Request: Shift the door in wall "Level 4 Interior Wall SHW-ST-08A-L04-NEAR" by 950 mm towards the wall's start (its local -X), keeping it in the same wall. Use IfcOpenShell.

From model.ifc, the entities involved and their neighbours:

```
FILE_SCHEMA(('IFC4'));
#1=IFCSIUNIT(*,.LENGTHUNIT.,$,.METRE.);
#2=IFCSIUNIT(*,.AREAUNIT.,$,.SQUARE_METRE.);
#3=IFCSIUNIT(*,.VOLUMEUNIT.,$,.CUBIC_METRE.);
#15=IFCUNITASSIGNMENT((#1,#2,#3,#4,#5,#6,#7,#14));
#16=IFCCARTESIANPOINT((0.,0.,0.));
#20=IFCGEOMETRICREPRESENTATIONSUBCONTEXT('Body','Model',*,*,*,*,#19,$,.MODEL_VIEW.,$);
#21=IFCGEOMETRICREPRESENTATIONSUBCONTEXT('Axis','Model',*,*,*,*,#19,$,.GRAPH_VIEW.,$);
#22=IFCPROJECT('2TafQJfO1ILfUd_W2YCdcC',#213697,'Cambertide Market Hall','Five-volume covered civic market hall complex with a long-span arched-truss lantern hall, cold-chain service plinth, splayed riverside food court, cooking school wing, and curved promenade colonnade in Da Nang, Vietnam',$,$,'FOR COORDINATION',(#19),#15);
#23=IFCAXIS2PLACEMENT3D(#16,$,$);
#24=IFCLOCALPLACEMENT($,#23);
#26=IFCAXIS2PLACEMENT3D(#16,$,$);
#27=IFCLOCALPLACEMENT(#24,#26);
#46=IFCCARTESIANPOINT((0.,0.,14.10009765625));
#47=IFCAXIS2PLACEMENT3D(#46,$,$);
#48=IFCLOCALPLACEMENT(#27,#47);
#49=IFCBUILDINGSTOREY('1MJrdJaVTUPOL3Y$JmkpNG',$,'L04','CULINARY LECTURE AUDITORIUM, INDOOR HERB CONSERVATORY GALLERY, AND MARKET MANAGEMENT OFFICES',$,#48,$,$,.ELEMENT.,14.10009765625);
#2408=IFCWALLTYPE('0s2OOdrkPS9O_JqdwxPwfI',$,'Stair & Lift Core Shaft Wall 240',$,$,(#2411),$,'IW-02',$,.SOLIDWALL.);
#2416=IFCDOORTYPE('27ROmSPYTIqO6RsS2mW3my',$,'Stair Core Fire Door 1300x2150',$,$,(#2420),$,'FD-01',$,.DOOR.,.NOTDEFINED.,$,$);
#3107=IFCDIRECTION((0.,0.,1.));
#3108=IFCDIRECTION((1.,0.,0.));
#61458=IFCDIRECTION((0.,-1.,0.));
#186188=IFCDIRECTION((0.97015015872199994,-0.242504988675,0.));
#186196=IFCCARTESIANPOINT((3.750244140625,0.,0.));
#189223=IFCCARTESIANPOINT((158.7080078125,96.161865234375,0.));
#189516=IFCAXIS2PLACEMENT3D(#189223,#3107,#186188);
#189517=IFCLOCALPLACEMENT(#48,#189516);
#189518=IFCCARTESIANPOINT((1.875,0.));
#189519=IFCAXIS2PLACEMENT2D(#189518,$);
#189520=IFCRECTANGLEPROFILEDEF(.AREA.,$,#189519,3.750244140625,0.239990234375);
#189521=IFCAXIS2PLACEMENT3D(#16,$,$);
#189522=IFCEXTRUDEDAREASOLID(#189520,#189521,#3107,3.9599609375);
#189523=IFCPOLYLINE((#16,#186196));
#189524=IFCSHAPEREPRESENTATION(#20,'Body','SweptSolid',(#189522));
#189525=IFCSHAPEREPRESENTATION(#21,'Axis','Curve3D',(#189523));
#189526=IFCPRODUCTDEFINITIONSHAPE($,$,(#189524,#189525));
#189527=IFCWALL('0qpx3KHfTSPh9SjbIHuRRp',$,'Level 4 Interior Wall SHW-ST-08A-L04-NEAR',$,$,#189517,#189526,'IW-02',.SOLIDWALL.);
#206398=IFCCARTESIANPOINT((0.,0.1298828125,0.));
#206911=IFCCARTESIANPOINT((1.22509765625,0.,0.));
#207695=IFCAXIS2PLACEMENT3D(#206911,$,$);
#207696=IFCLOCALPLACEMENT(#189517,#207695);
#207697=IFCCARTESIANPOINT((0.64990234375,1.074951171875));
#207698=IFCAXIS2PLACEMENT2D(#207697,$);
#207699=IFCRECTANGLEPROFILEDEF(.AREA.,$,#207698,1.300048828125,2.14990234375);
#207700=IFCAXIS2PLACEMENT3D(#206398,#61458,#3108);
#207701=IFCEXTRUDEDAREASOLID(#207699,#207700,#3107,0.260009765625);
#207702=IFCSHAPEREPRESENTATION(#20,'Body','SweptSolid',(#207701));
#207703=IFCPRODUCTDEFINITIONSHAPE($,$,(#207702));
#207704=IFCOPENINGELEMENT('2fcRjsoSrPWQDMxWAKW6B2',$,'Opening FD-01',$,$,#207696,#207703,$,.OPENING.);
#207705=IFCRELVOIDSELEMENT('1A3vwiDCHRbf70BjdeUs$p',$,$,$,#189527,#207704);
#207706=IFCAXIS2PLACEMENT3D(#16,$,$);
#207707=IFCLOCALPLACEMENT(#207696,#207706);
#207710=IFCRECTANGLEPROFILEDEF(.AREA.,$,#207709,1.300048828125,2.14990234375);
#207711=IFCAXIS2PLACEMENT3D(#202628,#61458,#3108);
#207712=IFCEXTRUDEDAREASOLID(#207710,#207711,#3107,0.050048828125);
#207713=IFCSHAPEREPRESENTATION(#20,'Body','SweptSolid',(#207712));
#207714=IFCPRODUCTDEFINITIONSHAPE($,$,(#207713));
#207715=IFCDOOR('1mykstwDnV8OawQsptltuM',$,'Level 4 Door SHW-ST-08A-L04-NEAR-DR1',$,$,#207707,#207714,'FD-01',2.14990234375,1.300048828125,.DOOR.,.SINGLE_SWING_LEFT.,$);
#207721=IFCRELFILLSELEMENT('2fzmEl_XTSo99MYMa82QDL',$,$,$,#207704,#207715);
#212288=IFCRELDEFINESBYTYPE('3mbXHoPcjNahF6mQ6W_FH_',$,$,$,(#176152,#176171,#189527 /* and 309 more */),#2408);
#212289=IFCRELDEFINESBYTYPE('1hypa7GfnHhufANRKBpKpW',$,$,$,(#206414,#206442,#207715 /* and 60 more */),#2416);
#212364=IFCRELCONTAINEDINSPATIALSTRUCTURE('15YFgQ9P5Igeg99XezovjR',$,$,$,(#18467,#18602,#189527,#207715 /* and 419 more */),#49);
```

```python
import ifcopenshell
import ifcopenshell.api.geometry
import ifcopenshell.util.placement
import ifcopenshell.util.unit

model = ifcopenshell.open("model.ifc")
unit_scale = ifcopenshell.util.unit.calculate_unit_scale(model)

door = model.by_id(207715)
opening = door.FillsVoids[0].RelatingOpeningElement
wall = opening.VoidsElements[0].RelatingBuildingElement

wall_matrix = ifcopenshell.util.placement.get_local_placement(wall.ObjectPlacement)
shift = wall_matrix[:3, 0] * -0.95 / unit_scale
before = ifcopenshell.util.placement.get_local_placement(door.ObjectPlacement)[:3, 3].copy()

# The door is placed relative to its opening, so it follows when the opening moves.
matrix = ifcopenshell.util.placement.get_local_placement(opening.ObjectPlacement)
matrix[:3, 3] += shift
ifcopenshell.api.geometry.edit_object_placement(
    model, product=opening, matrix=matrix, is_si=False, should_transform_children=True
)

after = ifcopenshell.util.placement.get_local_placement(door.ObjectPlacement)[:3, 3]
print("door moved by", (after - before).round(3) + 0.0)

model.write("model_rev.ifc")
```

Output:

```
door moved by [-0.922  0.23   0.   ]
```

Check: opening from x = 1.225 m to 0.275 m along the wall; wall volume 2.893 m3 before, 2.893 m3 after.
